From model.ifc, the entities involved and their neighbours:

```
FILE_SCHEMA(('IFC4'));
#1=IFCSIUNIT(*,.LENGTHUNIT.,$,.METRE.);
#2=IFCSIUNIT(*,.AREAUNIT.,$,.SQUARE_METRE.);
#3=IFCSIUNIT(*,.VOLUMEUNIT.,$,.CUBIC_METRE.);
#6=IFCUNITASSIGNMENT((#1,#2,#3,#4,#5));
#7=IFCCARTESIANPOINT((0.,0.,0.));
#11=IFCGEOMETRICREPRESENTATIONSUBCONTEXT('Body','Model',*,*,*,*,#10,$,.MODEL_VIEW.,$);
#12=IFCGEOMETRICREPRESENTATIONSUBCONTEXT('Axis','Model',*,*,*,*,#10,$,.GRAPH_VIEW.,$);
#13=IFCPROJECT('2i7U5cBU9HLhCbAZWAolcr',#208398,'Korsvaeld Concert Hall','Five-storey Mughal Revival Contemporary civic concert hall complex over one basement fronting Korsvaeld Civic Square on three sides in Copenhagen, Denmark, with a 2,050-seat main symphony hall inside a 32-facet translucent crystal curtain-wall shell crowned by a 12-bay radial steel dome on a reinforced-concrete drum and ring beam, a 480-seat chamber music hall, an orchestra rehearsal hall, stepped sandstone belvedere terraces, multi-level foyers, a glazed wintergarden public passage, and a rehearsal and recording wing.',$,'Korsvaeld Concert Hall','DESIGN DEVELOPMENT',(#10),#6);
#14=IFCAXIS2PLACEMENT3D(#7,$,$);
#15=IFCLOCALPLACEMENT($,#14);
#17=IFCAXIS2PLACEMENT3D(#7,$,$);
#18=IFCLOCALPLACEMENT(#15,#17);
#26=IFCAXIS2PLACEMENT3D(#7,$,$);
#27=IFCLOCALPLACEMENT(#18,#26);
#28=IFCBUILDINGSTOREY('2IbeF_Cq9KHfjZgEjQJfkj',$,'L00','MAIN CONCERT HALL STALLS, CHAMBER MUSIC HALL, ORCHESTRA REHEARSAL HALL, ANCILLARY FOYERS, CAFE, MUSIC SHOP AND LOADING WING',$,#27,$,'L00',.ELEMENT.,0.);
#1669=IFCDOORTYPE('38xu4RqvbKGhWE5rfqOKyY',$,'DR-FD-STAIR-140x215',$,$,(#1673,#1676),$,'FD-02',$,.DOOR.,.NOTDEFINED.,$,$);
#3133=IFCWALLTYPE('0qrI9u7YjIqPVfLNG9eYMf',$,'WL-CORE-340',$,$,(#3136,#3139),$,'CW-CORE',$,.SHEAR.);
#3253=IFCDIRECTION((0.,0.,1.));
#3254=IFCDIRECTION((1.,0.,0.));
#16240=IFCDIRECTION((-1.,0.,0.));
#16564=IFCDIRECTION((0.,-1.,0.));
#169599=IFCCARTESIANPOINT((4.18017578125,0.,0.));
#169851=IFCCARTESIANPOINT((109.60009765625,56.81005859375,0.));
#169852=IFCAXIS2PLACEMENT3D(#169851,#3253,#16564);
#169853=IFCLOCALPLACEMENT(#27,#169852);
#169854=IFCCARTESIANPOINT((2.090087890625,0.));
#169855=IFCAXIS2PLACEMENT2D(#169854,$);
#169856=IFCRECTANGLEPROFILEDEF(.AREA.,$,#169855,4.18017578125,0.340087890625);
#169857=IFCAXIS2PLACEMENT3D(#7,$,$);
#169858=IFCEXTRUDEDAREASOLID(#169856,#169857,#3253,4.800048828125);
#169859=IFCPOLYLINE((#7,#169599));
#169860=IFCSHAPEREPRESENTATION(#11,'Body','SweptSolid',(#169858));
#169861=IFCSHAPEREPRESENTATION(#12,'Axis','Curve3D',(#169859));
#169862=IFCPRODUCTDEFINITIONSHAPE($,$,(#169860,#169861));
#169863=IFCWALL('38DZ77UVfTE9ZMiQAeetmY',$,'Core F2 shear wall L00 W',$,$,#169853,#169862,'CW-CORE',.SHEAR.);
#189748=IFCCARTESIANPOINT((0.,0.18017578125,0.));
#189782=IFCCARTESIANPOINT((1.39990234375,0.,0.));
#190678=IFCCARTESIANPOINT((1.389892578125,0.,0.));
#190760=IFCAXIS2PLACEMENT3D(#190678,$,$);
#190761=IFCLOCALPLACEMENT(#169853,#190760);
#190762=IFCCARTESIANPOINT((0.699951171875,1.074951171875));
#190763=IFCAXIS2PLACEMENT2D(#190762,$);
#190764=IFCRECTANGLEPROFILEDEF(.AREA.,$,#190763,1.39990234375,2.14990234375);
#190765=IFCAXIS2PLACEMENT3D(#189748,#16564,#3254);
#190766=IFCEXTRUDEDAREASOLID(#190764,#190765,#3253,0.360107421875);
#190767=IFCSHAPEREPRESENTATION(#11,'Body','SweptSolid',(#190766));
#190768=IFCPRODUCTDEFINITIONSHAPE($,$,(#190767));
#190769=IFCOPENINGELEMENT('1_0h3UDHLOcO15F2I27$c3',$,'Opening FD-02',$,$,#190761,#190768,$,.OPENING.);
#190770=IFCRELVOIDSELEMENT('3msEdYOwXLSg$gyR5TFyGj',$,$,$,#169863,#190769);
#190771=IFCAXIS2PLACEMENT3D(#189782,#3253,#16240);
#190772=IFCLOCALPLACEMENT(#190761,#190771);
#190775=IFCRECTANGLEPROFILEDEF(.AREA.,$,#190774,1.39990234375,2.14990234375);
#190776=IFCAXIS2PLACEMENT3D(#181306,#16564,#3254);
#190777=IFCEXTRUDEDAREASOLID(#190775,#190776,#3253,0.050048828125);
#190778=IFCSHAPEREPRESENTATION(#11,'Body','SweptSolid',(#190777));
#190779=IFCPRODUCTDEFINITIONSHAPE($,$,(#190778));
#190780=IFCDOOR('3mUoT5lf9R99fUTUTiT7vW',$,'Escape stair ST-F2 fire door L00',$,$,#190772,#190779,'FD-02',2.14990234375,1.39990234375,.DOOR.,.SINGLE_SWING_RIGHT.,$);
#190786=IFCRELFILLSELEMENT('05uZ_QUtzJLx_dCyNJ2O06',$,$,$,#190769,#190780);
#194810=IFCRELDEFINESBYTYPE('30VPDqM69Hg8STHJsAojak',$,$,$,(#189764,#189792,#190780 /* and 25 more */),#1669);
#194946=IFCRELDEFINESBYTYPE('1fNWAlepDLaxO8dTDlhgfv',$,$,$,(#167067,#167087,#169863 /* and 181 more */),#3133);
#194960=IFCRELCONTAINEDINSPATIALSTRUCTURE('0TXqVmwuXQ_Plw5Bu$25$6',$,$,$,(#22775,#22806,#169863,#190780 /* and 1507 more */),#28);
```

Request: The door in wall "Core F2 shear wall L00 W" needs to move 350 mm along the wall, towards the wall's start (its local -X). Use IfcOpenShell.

```python
import ifcopenshell
import ifcopenshell.api.geometry
import ifcopenshell.util.placement
import ifcopenshell.util.unit

model = ifcopenshell.open("model.ifc")
unit_scale = ifcopenshell.util.unit.calculate_unit_scale(model)

door = model.by_guid("3mUoT5lf9R99fUTUTiT7vW")
opening = door.FillsVoids[0].RelatingOpeningElement
wall = opening.VoidsElements[0].RelatingBuildingElement

wall_matrix = ifcopenshell.util.placement.get_local_placement(wall.ObjectPlacement)
shift = wall_matrix[:3, 0] * -0.35 / unit_scale
before = ifcopenshell.util.placement.get_local_placement(door.ObjectPlacement)[:3, 3].copy()

# The door is placed relative to its opening, so it follows when the opening moves.
matrix = ifcopenshell.util.placement.get_local_placement(opening.ObjectPlacement)
matrix[:3, 3] += shift
ifcopenshell.api.geometry.edit_object_placement(
    model, product=opening, matrix=matrix, is_si=False, should_transform_children=True
)

after = ifcopenshell.util.placement.get_local_placement(door.ObjectPlacement)[:3, 3]
print("door moved by", (after - before).round(3) + 0.0)

model.write("model_v2.ifc")
```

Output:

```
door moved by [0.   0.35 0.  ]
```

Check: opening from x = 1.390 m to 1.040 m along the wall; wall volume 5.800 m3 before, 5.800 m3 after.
